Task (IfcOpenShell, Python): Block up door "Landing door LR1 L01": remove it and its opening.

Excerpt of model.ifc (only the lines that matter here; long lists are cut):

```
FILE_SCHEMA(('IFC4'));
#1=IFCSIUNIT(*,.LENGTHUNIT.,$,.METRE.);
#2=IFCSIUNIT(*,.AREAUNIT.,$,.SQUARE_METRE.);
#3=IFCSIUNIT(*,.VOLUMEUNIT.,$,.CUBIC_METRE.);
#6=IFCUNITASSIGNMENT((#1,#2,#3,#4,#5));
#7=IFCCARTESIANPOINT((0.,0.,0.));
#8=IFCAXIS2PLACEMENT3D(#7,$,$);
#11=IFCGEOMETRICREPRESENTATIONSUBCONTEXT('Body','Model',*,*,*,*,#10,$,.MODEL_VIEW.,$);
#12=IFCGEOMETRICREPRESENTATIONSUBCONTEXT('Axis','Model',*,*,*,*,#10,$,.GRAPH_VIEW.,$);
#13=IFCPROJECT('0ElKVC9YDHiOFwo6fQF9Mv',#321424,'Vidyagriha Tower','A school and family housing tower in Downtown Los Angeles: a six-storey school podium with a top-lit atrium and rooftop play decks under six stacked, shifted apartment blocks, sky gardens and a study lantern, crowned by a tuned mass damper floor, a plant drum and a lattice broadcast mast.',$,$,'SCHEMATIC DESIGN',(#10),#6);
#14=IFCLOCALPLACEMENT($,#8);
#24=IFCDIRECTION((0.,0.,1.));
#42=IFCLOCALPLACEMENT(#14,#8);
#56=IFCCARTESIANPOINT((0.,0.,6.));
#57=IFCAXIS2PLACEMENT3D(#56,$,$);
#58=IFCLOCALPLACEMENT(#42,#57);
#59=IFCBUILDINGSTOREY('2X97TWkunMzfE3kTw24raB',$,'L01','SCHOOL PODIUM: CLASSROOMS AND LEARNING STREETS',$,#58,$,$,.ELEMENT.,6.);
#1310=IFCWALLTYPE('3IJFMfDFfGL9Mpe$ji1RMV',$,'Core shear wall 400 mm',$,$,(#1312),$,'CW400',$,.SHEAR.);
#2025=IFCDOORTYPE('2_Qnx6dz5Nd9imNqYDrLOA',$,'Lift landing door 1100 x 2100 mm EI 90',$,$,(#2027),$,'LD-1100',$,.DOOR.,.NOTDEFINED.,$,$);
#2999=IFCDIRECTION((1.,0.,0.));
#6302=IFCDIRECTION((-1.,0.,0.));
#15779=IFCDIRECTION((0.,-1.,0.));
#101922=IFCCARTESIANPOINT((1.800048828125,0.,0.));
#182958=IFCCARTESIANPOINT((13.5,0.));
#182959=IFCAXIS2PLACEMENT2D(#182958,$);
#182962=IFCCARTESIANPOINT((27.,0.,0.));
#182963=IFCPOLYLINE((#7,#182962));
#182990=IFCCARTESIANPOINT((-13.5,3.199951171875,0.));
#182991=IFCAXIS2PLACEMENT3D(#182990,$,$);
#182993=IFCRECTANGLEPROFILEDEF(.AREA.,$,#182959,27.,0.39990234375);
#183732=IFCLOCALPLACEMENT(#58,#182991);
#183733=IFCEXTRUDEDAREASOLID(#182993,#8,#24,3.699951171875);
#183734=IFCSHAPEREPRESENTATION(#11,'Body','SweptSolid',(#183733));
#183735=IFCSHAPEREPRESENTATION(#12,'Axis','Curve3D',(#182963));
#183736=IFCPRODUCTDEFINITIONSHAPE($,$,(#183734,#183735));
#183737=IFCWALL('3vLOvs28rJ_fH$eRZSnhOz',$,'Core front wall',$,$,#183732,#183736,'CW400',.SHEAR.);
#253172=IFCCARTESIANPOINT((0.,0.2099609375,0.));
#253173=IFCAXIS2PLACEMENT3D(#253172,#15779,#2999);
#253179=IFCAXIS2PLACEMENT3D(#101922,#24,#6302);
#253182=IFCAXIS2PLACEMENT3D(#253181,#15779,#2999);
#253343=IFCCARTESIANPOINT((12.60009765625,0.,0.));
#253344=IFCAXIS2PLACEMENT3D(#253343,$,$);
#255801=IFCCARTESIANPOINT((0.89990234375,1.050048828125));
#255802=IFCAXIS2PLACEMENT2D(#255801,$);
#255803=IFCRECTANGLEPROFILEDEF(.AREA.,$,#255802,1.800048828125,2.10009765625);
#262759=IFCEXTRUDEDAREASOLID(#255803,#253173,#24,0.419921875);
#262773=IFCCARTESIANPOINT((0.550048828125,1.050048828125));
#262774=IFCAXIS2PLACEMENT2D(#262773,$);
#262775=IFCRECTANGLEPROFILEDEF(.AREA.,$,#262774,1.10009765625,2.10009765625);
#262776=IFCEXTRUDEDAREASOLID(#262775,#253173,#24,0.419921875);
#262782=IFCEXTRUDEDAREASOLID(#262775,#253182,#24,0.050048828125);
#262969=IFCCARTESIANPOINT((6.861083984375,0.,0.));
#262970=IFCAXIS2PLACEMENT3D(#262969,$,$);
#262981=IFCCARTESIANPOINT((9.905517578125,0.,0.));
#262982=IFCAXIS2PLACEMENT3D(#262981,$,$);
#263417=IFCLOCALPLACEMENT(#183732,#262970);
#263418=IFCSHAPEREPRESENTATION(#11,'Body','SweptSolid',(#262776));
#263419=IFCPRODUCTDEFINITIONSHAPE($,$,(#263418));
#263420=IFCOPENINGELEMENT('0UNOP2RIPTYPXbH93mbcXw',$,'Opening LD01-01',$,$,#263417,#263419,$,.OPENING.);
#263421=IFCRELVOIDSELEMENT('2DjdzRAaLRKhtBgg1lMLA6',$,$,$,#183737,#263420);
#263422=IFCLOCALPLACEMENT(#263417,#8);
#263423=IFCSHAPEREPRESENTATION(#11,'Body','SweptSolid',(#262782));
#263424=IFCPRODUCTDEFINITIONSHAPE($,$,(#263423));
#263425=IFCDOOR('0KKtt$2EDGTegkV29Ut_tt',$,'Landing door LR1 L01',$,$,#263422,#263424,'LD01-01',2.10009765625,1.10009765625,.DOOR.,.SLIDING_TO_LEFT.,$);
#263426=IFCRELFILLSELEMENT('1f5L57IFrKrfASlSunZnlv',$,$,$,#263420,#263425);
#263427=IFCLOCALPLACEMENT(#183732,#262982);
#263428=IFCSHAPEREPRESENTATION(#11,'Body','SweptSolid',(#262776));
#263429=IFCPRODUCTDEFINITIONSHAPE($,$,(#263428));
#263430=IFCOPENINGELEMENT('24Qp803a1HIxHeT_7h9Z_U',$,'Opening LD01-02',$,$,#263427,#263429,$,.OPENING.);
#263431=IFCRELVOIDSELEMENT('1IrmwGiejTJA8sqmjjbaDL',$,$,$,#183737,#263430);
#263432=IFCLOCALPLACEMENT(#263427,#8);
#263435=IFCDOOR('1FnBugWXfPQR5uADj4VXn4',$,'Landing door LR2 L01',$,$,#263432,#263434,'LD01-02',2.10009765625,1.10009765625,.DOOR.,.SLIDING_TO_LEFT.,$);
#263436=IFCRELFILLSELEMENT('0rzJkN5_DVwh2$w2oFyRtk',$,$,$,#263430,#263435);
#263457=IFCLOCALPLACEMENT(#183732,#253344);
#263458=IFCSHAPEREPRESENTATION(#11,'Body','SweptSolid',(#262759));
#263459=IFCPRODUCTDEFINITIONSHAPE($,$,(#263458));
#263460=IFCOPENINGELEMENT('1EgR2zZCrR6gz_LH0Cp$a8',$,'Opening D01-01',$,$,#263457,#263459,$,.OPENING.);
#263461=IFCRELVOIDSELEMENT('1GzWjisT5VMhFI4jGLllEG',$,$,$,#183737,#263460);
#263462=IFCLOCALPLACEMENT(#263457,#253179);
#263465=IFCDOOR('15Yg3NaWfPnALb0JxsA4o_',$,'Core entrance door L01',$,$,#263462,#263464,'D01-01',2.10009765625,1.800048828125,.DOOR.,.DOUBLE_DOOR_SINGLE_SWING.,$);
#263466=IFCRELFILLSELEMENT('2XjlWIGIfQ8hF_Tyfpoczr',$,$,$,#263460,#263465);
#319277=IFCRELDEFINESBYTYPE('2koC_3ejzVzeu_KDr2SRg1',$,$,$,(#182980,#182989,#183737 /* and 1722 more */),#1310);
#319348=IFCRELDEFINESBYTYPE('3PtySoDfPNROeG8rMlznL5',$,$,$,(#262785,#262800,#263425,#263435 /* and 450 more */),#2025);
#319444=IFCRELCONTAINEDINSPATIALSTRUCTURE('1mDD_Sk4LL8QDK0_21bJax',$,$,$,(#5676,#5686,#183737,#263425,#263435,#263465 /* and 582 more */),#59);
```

```python
import ifcopenshell
import ifcopenshell.api.feature
import ifcopenshell.api.root
import ifcopenshell.geom
import ifcopenshell.util.shape

model = ifcopenshell.open("model.ifc")
settings = ifcopenshell.geom.settings()


def volume(element):
    """Net volume in cubic metres, openings subtracted."""
    shape = ifcopenshell.geom.create_shape(settings, element)
    return ifcopenshell.util.shape.get_volume(shape.geometry)


door = model.by_guid("0KKtt$2EDGTegkV29Ut_tt")
opening = door.FillsVoids[0].RelatingOpeningElement
wall = opening.VoidsElements[0].RelatingBuildingElement
before = volume(wall)

ifcopenshell.api.root.remove_product(model, product=door)
ifcopenshell.api.feature.remove_feature(model, feature=opening)

after = volume(wall)

print(f"wall volume {before:.3f} -> {after:.3f} m3")

model.write("model_updated.ifc")
```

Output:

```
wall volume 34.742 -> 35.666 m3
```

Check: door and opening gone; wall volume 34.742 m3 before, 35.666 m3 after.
